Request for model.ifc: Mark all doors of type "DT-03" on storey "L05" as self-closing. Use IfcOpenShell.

First a look at what the model holds.

```python
import ifcopenshell
import ifcopenshell.util.element

model = ifcopenshell.open("model.ifc")
print(model.schema)
storey = next(s for s in model.by_type("IfcBuildingStorey") if s.Name == "L05")
doors = [e for e in ifcopenshell.util.element.get_decomposition(storey) if e.is_a("IfcDoor")]
seen = {}
for e in doors:
    element_type = ifcopenshell.util.element.get_type(e)
    key = (element_type.Name if element_type != e and element_type else None, ifcopenshell.util.element.get_pset(e, "Pset_DoorCommon", "SelfClosing"))
    seen[key] = seen.get(key, 0) + 1
for (name, value), count in sorted(seen.items(), key=str):
    print(count, "x", name, "|", value)
```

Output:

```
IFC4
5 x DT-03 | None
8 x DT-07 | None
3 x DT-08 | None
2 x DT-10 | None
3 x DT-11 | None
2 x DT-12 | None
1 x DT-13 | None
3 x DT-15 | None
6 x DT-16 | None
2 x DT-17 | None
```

```python
import ifcopenshell
import ifcopenshell.api.pset
import ifcopenshell.util.element

model = ifcopenshell.open("model.ifc")

storey = next(s for s in model.by_type("IfcBuildingStorey") if s.Name == "L05")
doors = [e for e in ifcopenshell.util.element.get_decomposition(storey) if e.is_a("IfcDoor")]

count = 0
for e in doors:
    element_type = ifcopenshell.util.element.get_type(e)
    if element_type in (None, e) or element_type.Name != "DT-03":
        continue
    # add_pset returns the element's existing set when there is one.
    pset = ifcopenshell.api.pset.add_pset(model, product=e, name="Pset_DoorCommon")
    ifcopenshell.api.pset.edit_pset(model, pset=pset, properties={"SelfClosing": True})
    count += 1

print(count, "doors updated")

model.write("model_rev.ifc")
```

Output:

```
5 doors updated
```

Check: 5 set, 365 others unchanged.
